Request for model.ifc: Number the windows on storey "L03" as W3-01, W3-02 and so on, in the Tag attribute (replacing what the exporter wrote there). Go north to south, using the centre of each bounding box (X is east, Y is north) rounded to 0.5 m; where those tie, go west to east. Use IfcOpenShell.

First a look at what the model holds.

```python
import ifcopenshell
import ifcopenshell.util.element
import ifcopenshell.util.placement

model = ifcopenshell.open("model.ifc")
print(model.schema)
storey = next(s for s in model.by_type("IfcBuildingStorey") if s.Name == "L03")
windows = [e for e in ifcopenshell.util.element.get_decomposition(storey) if e.is_a("IfcWindow")]
for e in sorted(windows, key=lambda e: e.id()):
    origin = ifcopenshell.util.placement.get_local_placement(e.ObjectPlacement)[:3, 3]
    print(e.id(), e.Tag, e.Name, origin.round(2) + 0.0, sep=" | ")
```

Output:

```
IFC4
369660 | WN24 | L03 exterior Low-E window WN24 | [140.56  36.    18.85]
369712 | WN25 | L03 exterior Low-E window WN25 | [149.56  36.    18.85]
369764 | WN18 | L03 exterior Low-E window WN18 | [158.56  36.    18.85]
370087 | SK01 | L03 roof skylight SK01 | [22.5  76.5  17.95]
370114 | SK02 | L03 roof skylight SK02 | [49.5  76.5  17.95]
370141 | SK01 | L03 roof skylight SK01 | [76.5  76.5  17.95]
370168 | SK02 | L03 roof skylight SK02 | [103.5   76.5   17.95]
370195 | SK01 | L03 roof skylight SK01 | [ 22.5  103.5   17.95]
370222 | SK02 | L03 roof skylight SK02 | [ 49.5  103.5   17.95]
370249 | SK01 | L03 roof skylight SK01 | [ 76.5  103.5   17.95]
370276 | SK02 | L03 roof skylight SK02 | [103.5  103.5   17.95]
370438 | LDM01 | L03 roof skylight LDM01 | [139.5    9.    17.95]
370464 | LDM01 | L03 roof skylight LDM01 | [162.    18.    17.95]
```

```python
import ifcopenshell
import ifcopenshell.geom
import ifcopenshell.util.element
import ifcopenshell.util.shape

model = ifcopenshell.open("model.ifc")
settings = ifcopenshell.geom.settings()
settings.set("use-world-coords", True)


def centre(element):
    shape = ifcopenshell.geom.create_shape(settings, element)
    return ifcopenshell.util.shape.get_bbox_centroid(shape.geometry)


storey = next(s for s in model.by_type("IfcBuildingStorey") if s.Name == "L03")
windows = [e for e in ifcopenshell.util.element.get_decomposition(storey) if e.is_a("IfcWindow")]

# Insertion points can sit at a corner or the storey origin, so sort by the geometry (in metres).
centres = {e: centre(e) for e in windows}
windows.sort(key=lambda e: (-round(centres[e][1] / 0.5), centres[e][0]))

for i, e in enumerate(windows, start=1):
    number = f"W3-{i:02d}"
    e.Tag = number
    print(e.id(), number)

model.write("model_rev.ifc")
```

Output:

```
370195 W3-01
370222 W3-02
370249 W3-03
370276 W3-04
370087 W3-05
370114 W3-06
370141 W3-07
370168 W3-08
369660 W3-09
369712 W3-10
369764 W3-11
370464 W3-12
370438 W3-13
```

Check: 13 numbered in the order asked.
